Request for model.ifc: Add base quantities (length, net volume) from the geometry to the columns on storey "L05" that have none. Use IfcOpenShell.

First a look at what the model holds.

```python
import ifcopenshell
import ifcopenshell.util.element
import ifcopenshell.util.unit

model = ifcopenshell.open("model.ifc")
print(model.schema)
for unit_type in ("LENGTHUNIT", "AREAUNIT", "VOLUMEUNIT"):
    print(unit_type, ifcopenshell.util.unit.calculate_unit_scale(model, unit_type))
storey = next(s for s in model.by_type("IfcBuildingStorey") if s.Name == "L05")
columns = [e for e in ifcopenshell.util.element.get_decomposition(storey) if e.is_a("IfcColumn")]
for e in sorted(columns, key=lambda e: e.id()):
    print(e.id(), e.is_a(), e.Name, list(ifcopenshell.util.element.get_psets(e, qtos_only=True)), sep=" | ")
```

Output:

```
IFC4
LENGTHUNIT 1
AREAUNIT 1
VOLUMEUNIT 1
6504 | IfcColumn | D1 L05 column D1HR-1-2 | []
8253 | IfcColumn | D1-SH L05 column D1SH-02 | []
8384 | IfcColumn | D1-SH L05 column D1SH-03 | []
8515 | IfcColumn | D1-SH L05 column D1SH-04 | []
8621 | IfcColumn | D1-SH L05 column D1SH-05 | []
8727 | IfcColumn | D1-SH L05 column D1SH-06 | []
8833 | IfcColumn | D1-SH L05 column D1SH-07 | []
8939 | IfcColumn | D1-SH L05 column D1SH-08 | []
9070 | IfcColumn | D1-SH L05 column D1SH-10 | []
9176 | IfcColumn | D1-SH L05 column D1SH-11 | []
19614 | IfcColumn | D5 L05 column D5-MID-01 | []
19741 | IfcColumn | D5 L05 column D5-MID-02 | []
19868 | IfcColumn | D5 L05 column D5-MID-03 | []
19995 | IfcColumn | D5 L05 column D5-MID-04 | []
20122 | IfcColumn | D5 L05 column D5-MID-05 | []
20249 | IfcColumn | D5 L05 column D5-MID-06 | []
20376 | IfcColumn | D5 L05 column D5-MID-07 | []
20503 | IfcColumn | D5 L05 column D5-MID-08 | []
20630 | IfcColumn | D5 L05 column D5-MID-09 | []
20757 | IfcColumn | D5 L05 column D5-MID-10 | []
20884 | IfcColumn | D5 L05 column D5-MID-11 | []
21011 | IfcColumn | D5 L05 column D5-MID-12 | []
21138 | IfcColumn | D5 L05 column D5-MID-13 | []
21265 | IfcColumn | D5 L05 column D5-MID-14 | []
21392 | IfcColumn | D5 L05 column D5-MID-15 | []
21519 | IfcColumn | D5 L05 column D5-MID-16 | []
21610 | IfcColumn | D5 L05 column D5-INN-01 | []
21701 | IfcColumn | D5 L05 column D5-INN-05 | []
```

```python
import ifcopenshell
import ifcopenshell.api.pset
import ifcopenshell.geom
import ifcopenshell.util.element
import ifcopenshell.util.shape
import ifcopenshell.util.unit

model = ifcopenshell.open("model.ifc")
unit_scale = ifcopenshell.util.unit.calculate_unit_scale(model)
volume_scale = ifcopenshell.util.unit.calculate_unit_scale(model, "VOLUMEUNIT")
settings = ifcopenshell.geom.settings()

storey = next(s for s in model.by_type("IfcBuildingStorey") if s.Name == "L05")
columns = [e for e in ifcopenshell.util.element.get_decomposition(storey) if e.is_a("IfcColumn")]

for e in sorted(columns, key=lambda e: e.id()):
    if ifcopenshell.util.element.get_psets(e, qtos_only=True, should_inherit=False):
        continue
    # Geometry comes back in metres, in the element's own axes.
    shape = ifcopenshell.geom.create_shape(settings, e)
    values = {
        "Length": ifcopenshell.util.shape.get_z(shape.geometry) / unit_scale,
        "NetVolume": ifcopenshell.util.shape.get_volume(shape.geometry) / volume_scale,
    }
    qto = ifcopenshell.api.pset.add_qto(model, product=e, name="Qto_ColumnBaseQuantities")
    ifcopenshell.api.pset.edit_qto(model, qto=qto, properties=values)
    print(e.id(), {k: round(v, 3) for k, v in values.items()})

model.write("model_v2.ifc")
```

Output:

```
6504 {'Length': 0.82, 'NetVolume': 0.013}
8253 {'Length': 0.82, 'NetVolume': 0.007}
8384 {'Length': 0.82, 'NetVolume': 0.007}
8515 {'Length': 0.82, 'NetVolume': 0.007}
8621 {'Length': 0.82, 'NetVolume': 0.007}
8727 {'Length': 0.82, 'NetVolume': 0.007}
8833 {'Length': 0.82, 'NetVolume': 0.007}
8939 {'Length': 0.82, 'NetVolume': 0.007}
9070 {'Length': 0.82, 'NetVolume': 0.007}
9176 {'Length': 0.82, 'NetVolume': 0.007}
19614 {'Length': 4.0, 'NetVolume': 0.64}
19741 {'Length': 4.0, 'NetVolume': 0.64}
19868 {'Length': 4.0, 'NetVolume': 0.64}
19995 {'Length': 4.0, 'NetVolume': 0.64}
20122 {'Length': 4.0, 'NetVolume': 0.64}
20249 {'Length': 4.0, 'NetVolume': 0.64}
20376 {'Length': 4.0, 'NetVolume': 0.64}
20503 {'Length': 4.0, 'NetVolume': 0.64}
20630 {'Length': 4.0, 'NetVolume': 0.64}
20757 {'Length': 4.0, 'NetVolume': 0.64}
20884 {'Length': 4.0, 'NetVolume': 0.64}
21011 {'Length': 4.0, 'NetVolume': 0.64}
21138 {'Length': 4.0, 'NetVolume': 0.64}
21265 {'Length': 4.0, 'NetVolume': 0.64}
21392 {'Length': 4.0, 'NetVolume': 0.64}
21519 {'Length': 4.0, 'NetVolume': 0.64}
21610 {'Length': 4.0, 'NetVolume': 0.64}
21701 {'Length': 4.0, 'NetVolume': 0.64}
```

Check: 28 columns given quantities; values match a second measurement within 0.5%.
